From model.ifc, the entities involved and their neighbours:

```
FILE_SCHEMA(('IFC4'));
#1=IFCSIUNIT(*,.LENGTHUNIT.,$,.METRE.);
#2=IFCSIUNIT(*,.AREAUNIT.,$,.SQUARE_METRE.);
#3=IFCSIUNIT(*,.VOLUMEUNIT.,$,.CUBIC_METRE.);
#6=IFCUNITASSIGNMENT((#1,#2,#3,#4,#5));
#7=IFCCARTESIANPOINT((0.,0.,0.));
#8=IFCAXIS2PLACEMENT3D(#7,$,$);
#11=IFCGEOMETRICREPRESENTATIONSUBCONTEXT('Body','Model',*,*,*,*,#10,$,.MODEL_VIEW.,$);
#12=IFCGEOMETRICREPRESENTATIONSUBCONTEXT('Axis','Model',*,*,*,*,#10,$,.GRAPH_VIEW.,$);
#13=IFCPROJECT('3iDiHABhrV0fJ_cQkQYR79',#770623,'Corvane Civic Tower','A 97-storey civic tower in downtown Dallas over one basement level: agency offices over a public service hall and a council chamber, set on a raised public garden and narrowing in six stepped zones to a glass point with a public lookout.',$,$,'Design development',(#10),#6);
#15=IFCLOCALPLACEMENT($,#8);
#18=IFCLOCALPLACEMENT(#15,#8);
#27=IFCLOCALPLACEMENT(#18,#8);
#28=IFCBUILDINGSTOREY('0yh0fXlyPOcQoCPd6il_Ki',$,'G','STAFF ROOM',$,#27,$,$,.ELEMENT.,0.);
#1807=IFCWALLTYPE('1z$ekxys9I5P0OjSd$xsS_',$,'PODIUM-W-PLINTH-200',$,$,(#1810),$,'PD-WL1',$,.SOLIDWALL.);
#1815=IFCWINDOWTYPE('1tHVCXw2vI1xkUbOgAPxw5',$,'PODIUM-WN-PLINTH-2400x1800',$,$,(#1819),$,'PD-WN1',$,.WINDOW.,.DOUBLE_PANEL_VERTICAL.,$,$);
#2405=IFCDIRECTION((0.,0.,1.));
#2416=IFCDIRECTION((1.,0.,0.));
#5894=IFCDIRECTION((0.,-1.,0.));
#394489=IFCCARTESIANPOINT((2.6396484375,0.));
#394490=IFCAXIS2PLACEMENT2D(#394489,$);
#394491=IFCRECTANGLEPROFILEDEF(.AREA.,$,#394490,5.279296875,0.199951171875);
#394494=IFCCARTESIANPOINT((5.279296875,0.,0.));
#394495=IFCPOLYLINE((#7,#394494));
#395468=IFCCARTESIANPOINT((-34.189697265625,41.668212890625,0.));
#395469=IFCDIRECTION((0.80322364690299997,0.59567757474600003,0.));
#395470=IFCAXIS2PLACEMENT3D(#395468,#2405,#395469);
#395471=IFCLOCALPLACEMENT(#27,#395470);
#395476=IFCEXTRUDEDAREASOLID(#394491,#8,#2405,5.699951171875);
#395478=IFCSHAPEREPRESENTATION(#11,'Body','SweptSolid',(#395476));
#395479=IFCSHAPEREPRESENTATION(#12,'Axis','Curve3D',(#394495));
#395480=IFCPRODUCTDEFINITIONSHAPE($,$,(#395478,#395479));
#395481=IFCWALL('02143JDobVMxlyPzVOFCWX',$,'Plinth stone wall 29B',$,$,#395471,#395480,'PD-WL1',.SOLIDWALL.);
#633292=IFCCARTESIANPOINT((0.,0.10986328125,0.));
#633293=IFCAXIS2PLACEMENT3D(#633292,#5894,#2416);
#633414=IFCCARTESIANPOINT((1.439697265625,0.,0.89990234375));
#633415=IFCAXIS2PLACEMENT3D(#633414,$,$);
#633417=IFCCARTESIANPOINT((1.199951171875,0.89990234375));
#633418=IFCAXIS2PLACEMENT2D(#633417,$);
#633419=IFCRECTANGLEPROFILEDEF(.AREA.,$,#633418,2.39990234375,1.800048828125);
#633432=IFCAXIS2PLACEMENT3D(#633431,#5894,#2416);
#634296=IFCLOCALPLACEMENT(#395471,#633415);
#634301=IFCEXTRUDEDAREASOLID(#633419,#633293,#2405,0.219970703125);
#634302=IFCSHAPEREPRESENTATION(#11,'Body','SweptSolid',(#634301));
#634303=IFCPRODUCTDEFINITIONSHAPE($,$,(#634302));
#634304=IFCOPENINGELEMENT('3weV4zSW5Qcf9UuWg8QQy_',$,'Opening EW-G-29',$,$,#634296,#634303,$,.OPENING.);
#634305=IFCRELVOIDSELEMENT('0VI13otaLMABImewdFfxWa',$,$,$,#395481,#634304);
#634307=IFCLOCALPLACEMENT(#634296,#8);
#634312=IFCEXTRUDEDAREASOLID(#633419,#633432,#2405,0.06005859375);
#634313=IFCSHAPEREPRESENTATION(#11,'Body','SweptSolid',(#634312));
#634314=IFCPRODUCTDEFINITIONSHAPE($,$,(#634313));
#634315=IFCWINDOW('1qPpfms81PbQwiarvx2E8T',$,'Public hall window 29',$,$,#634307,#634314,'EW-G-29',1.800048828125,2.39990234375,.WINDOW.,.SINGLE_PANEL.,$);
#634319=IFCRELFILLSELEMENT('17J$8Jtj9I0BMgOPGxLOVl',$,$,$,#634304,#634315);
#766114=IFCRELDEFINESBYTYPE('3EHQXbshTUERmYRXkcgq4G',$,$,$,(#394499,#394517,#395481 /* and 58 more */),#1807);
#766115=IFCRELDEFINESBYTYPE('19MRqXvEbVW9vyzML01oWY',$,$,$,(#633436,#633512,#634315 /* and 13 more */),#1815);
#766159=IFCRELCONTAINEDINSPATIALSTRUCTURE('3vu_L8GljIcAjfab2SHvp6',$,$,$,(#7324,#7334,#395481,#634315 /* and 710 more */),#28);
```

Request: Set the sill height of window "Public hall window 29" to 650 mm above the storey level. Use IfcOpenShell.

```python
import numpy as np
import ifcopenshell
import ifcopenshell.api.geometry
import ifcopenshell.geom
import ifcopenshell.util.element
import ifcopenshell.util.placement
import ifcopenshell.util.shape
import ifcopenshell.util.unit

model = ifcopenshell.open("model.ifc")
unit_scale = ifcopenshell.util.unit.calculate_unit_scale(model)

window = model.by_id(634315)
opening = window.FillsVoids[0].RelatingOpeningElement
storey = ifcopenshell.util.element.get_container(window, ifc_class="IfcBuildingStorey")
level = ifcopenshell.util.placement.get_local_placement(storey.ObjectPlacement)[2, 3]

# The opening's origin need not be at the sill, so measure its lowest point.
shape = ifcopenshell.geom.create_shape(ifcopenshell.geom.settings(), opening)
bottom = ifcopenshell.util.shape.get_shape_bottom_elevation(shape, shape.geometry) / unit_scale
dz = level + 0.65 - bottom

shift = np.array([0.0, 0.0, dz])
# The window is placed relative to its opening, so it follows when the opening moves.
matrix = ifcopenshell.util.placement.get_local_placement(opening.ObjectPlacement)
matrix[:3, 3] += shift
ifcopenshell.api.geometry.edit_object_placement(
    model, product=opening, matrix=matrix, is_si=False, should_transform_children=True
)

print(f"moved by {dz * unit_scale:+.3f} m")

model.write("model_v2.ifc")
```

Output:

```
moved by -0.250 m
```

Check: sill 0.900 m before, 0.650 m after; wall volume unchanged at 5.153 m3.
